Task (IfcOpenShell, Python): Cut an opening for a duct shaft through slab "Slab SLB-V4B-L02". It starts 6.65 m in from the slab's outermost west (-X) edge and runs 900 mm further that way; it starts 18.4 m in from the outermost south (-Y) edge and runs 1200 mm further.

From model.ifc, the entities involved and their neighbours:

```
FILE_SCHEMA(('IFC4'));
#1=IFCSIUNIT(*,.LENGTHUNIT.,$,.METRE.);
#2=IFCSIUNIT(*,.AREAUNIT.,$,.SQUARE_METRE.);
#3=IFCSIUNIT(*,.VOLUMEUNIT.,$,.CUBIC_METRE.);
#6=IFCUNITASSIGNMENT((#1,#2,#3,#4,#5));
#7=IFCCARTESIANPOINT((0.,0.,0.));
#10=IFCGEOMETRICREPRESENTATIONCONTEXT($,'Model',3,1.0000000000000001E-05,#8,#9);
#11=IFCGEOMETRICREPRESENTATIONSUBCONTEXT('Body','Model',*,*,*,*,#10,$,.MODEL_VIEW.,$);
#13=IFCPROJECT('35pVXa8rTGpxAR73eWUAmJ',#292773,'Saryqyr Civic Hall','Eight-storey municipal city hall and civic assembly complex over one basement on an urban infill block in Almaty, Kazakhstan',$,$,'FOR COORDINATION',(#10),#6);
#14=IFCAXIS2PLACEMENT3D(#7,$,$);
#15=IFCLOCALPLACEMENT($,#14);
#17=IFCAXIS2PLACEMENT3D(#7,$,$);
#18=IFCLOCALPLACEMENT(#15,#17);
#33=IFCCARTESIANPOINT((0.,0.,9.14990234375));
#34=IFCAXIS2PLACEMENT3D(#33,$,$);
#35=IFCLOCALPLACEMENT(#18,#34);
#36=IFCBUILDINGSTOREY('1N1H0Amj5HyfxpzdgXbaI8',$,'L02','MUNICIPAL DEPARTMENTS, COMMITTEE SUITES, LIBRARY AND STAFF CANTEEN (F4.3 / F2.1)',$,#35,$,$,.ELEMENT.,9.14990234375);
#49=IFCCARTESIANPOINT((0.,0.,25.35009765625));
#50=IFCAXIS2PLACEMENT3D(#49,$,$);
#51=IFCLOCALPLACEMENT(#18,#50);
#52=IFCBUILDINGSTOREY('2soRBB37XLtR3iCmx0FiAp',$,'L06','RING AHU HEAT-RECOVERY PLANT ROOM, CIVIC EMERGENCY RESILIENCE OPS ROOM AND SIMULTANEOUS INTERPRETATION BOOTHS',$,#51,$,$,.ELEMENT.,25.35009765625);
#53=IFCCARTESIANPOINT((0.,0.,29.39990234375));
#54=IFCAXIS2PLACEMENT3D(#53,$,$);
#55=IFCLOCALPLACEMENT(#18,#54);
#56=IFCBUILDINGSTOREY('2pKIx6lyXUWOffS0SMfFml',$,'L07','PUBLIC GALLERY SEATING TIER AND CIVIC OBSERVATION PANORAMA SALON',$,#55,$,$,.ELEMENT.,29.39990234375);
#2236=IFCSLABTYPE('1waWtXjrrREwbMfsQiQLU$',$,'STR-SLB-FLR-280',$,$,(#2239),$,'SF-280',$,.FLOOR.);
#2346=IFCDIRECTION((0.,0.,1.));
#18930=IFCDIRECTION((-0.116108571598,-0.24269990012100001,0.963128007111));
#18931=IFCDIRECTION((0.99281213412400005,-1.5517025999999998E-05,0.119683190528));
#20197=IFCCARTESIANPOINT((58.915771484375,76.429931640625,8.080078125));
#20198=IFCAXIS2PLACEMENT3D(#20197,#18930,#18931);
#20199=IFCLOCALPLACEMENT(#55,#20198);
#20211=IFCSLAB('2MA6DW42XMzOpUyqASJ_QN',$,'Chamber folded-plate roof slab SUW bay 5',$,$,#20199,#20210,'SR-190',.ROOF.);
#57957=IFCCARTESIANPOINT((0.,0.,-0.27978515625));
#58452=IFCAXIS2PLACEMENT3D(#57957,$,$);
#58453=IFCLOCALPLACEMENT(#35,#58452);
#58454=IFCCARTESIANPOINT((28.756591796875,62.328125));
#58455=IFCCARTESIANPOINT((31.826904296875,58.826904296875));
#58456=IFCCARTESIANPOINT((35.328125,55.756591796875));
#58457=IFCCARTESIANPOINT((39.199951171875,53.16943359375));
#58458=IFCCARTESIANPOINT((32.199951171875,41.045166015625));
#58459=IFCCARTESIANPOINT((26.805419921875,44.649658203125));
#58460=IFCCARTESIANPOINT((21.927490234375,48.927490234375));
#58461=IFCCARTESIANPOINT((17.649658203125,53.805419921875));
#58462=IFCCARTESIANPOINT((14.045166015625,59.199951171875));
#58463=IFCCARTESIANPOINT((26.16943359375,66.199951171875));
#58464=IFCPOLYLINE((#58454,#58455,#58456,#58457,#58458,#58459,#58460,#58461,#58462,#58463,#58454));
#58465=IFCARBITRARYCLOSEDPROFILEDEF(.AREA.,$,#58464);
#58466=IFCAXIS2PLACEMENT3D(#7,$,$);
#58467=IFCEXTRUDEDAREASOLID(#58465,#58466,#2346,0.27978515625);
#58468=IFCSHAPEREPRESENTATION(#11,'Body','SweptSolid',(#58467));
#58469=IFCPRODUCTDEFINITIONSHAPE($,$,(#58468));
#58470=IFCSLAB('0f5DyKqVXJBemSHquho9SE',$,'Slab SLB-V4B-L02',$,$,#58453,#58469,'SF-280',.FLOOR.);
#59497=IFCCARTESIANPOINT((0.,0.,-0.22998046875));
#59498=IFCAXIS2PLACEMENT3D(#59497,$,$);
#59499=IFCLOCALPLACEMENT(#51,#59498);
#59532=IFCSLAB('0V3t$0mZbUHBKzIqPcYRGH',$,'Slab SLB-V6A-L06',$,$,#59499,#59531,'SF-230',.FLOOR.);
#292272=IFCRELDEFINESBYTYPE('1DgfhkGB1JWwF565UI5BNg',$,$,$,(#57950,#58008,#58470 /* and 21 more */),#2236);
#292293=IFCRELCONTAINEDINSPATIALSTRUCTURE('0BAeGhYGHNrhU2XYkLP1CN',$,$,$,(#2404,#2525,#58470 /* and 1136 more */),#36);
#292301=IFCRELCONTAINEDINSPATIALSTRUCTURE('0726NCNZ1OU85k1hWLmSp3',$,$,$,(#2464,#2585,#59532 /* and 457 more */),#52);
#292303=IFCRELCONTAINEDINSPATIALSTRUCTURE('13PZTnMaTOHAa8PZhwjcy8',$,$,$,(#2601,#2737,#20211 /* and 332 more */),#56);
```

```python
import numpy as np
import ifcopenshell
import ifcopenshell.api.feature
import ifcopenshell.api.geometry
import ifcopenshell.api.root
import ifcopenshell.geom
import ifcopenshell.util.placement
import ifcopenshell.util.representation
import ifcopenshell.util.shape
import ifcopenshell.util.unit

model = ifcopenshell.open("model.ifc")
unit_scale = ifcopenshell.util.unit.calculate_unit_scale(model)
settings = ifcopenshell.geom.settings()


def volume(element):
    """Net volume in cubic metres, openings subtracted."""
    shape = ifcopenshell.geom.create_shape(settings, element)
    return ifcopenshell.util.shape.get_volume(shape.geometry)


slab = model.by_id(58470)
before = volume(slab)

# Extent in the slab's own axes, in metres. The edges named are its -X and -Y sides.
slab_shape = ifcopenshell.geom.create_shape(settings, slab)
vertices = ifcopenshell.util.shape.get_vertices(slab_shape.geometry)
x_min, y_min, bottom = vertices.min(axis=0)
top = vertices[:, 2].max()

opening = ifcopenshell.api.root.create_entity(model, ifc_class="IfcOpeningElement", name="Duct shaft opening", predefined_type="OPENING")
context = ifcopenshell.util.representation.get_context(model, "Model", "Body", "MODEL_VIEW")
width, depth = 0.9, 1.2
outline = [(0.0, 0.0), (width, 0.0), (width, depth), (0.0, depth), (0.0, 0.0)]
# Overshoot both faces by 50 mm so the cut is clean.
shape = ifcopenshell.api.geometry.add_slab_representation(
    model, context=context, depth=top - bottom + 0.1, polyline=outline
)
ifcopenshell.api.geometry.assign_representation(model, product=opening, representation=shape)

matrix = ifcopenshell.util.placement.get_local_placement(slab.ObjectPlacement)
matrix[:, 3] = matrix @ np.append(np.array([x_min + 6.65, y_min + 18.4, bottom - 0.05]) / unit_scale, 1.0)
ifcopenshell.api.geometry.edit_object_placement(model, product=opening, matrix=matrix, is_si=False)
ifcopenshell.api.feature.add_feature(model, feature=opening, element=slab)

after = volume(slab)

print(f"slab volume {before:.3f} -> {after:.3f} m3")

model.write("model_v2.ifc")
```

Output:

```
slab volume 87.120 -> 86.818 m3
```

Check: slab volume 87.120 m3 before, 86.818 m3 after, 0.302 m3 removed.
